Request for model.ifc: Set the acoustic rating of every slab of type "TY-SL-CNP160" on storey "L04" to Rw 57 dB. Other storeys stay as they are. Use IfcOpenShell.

First a look at what the model holds.

```python
import ifcopenshell
import ifcopenshell.util.element

model = ifcopenshell.open("model.ifc")
print(model.schema)
storey = next(s for s in model.by_type("IfcBuildingStorey") if s.Name == "L04")
slabs = [e for e in ifcopenshell.util.element.get_decomposition(storey) if e.is_a("IfcSlab")]
seen = {}
for e in slabs:
    element_type = ifcopenshell.util.element.get_type(e)
    key = (element_type.Name if element_type != e and element_type else None, ifcopenshell.util.element.get_pset(e, "Pset_SlabCommon", "AcousticRating"))
    seen[key] = seen.get(key, 0) + 1
for (name, value), count in sorted(seen.items(), key=str):
    print(count, "x", name, "|", value)
```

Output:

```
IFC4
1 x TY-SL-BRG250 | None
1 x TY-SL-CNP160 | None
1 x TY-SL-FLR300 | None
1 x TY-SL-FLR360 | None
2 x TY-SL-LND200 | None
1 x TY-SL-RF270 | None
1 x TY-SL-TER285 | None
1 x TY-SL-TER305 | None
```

```python
import ifcopenshell
import ifcopenshell.api.pset
import ifcopenshell.util.element

model = ifcopenshell.open("model.ifc")

storey = next(s for s in model.by_type("IfcBuildingStorey") if s.Name == "L04")
slabs = [e for e in ifcopenshell.util.element.get_decomposition(storey) if e.is_a("IfcSlab")]

count = 0
for e in slabs:
    element_type = ifcopenshell.util.element.get_type(e)
    if element_type in (None, e) or element_type.Name != "TY-SL-CNP160":
        continue
    # add_pset returns the element's existing set when there is one.
    pset = ifcopenshell.api.pset.add_pset(model, product=e, name="Pset_SlabCommon")
    ifcopenshell.api.pset.edit_pset(model, pset=pset, properties={"AcousticRating": "Rw 57 dB"})
    count += 1

print(count, "slabs updated")

model.write("model_updated.ifc")
```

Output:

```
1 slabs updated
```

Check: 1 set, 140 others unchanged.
